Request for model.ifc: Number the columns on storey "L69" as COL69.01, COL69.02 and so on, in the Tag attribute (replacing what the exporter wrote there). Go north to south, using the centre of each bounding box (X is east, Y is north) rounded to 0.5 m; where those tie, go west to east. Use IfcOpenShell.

First a look at what the model holds.

```python
import ifcopenshell
import ifcopenshell.util.element
import ifcopenshell.util.placement

model = ifcopenshell.open("model.ifc")
print(model.schema)
storey = next(s for s in model.by_type("IfcBuildingStorey") if s.Name == "L69")
columns = [e for e in ifcopenshell.util.element.get_decomposition(storey) if e.is_a("IfcColumn")]
for e in sorted(columns, key=lambda e: e.id()):
    origin = ifcopenshell.util.placement.get_local_placement(e.ObjectPlacement)[:3, 3]
    print(e.id(), e.Tag, e.Name, origin.round(2) + 0.0, sep=" | ")
```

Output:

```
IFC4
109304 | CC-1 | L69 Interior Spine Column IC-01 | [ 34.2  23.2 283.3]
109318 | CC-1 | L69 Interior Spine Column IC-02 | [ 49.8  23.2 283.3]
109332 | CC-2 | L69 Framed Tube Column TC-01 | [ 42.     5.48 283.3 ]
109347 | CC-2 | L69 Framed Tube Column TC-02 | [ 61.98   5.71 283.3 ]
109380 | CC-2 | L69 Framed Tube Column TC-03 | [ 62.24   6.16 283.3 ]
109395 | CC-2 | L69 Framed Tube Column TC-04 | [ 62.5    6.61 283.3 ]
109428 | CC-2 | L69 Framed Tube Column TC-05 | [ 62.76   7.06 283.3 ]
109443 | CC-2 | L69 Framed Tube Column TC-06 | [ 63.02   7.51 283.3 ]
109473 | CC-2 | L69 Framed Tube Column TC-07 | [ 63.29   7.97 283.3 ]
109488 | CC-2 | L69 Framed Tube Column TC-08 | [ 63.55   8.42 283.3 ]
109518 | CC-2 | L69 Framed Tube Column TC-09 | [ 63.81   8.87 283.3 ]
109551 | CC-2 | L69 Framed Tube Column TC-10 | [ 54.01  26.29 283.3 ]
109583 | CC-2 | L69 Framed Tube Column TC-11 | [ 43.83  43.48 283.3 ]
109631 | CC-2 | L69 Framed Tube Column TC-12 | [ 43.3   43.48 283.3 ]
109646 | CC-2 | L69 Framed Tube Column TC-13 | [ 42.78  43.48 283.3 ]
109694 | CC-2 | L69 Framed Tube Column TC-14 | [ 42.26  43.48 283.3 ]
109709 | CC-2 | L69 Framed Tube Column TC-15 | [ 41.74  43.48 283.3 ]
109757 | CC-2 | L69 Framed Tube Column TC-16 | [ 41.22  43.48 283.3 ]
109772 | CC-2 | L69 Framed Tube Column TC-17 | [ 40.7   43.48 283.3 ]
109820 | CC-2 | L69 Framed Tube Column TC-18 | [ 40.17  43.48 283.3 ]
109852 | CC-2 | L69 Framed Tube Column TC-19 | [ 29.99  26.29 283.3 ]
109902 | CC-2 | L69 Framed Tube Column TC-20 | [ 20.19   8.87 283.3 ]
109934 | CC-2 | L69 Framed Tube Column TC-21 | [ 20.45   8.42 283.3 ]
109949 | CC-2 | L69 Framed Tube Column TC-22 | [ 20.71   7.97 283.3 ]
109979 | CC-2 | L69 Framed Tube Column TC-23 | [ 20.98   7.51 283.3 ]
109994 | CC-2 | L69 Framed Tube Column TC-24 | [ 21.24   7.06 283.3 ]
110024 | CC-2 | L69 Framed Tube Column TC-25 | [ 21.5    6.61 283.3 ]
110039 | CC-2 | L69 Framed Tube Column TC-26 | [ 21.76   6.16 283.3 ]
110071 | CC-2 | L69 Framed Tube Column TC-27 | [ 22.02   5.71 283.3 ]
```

```python
import ifcopenshell
import ifcopenshell.geom
import ifcopenshell.util.element
import ifcopenshell.util.shape

model = ifcopenshell.open("model.ifc")
settings = ifcopenshell.geom.settings()
settings.set("use-world-coords", True)


def centre(element):
    shape = ifcopenshell.geom.create_shape(settings, element)
    return ifcopenshell.util.shape.get_bbox_centroid(shape.geometry)


storey = next(s for s in model.by_type("IfcBuildingStorey") if s.Name == "L69")
columns = [e for e in ifcopenshell.util.element.get_decomposition(storey) if e.is_a("IfcColumn")]

# Insertion points can sit at a corner or the storey origin, so sort by the geometry (in metres).
centres = {e: centre(e) for e in columns}
columns.sort(key=lambda e: (-round(centres[e][1] / 0.5), centres[e][0]))

for i, e in enumerate(columns, start=1):
    number = f"COL69.{i:02d}"
    e.Tag = number
    print(e.id(), number)

model.write("model_v2.ifc")
```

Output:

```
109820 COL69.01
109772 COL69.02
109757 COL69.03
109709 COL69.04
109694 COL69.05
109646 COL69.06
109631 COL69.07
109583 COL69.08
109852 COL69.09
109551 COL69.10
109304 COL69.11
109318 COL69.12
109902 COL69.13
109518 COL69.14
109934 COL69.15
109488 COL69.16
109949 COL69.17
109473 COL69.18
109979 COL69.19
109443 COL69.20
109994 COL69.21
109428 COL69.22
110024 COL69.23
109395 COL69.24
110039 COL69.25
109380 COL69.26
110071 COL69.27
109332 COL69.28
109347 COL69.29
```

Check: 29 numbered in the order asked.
